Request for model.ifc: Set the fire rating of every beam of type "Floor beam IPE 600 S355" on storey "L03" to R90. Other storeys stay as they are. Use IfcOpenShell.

First a look at what the model holds.

```python
import ifcopenshell
import ifcopenshell.util.element

model = ifcopenshell.open("model.ifc")
print(model.schema)
storey = next(s for s in model.by_type("IfcBuildingStorey") if s.Name == "L03")
beams = [e for e in ifcopenshell.util.element.get_decomposition(storey) if e.is_a("IfcBeam")]
seen = {}
for e in beams:
    element_type = ifcopenshell.util.element.get_type(e)
    key = (element_type.Name if element_type != e and element_type else None, ifcopenshell.util.element.get_pset(e, "Pset_BeamCommon", "FireRating"))
    seen[key] = seen.get(key, 0) + 1
for (name, value), count in sorted(seen.items(), key=str):
    print(count, "x", name, "|", value)
```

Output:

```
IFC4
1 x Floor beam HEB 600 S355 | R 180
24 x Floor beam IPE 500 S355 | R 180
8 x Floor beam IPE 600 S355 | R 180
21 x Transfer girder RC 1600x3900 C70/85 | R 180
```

```python
import ifcopenshell
import ifcopenshell.api.pset
import ifcopenshell.util.element

model = ifcopenshell.open("model.ifc")

storey = next(s for s in model.by_type("IfcBuildingStorey") if s.Name == "L03")
beams = [e for e in ifcopenshell.util.element.get_decomposition(storey) if e.is_a("IfcBeam")]

count = 0
for e in beams:
    element_type = ifcopenshell.util.element.get_type(e)
    if element_type in (None, e) or element_type.Name != "Floor beam IPE 600 S355":
        continue
    found = ifcopenshell.util.element.get_pset(e, "Pset_BeamCommon", should_inherit=False)
    if found:
        pset = model.by_id(found["id"])
        if len(ifcopenshell.util.element.get_elements_by_pset(pset)) > 1:
            pset = ifcopenshell.api.pset.unshare_pset(model, products=[e], pset=pset)[0]
    else:
        pset = ifcopenshell.api.pset.add_pset(model, product=e, name="Pset_BeamCommon")
    ifcopenshell.api.pset.edit_pset(model, pset=pset, properties={"FireRating": "R90"})
    count += 1

print(count, "beams updated")

model.write("model-out.ifc")
```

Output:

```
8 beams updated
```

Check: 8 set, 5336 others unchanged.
